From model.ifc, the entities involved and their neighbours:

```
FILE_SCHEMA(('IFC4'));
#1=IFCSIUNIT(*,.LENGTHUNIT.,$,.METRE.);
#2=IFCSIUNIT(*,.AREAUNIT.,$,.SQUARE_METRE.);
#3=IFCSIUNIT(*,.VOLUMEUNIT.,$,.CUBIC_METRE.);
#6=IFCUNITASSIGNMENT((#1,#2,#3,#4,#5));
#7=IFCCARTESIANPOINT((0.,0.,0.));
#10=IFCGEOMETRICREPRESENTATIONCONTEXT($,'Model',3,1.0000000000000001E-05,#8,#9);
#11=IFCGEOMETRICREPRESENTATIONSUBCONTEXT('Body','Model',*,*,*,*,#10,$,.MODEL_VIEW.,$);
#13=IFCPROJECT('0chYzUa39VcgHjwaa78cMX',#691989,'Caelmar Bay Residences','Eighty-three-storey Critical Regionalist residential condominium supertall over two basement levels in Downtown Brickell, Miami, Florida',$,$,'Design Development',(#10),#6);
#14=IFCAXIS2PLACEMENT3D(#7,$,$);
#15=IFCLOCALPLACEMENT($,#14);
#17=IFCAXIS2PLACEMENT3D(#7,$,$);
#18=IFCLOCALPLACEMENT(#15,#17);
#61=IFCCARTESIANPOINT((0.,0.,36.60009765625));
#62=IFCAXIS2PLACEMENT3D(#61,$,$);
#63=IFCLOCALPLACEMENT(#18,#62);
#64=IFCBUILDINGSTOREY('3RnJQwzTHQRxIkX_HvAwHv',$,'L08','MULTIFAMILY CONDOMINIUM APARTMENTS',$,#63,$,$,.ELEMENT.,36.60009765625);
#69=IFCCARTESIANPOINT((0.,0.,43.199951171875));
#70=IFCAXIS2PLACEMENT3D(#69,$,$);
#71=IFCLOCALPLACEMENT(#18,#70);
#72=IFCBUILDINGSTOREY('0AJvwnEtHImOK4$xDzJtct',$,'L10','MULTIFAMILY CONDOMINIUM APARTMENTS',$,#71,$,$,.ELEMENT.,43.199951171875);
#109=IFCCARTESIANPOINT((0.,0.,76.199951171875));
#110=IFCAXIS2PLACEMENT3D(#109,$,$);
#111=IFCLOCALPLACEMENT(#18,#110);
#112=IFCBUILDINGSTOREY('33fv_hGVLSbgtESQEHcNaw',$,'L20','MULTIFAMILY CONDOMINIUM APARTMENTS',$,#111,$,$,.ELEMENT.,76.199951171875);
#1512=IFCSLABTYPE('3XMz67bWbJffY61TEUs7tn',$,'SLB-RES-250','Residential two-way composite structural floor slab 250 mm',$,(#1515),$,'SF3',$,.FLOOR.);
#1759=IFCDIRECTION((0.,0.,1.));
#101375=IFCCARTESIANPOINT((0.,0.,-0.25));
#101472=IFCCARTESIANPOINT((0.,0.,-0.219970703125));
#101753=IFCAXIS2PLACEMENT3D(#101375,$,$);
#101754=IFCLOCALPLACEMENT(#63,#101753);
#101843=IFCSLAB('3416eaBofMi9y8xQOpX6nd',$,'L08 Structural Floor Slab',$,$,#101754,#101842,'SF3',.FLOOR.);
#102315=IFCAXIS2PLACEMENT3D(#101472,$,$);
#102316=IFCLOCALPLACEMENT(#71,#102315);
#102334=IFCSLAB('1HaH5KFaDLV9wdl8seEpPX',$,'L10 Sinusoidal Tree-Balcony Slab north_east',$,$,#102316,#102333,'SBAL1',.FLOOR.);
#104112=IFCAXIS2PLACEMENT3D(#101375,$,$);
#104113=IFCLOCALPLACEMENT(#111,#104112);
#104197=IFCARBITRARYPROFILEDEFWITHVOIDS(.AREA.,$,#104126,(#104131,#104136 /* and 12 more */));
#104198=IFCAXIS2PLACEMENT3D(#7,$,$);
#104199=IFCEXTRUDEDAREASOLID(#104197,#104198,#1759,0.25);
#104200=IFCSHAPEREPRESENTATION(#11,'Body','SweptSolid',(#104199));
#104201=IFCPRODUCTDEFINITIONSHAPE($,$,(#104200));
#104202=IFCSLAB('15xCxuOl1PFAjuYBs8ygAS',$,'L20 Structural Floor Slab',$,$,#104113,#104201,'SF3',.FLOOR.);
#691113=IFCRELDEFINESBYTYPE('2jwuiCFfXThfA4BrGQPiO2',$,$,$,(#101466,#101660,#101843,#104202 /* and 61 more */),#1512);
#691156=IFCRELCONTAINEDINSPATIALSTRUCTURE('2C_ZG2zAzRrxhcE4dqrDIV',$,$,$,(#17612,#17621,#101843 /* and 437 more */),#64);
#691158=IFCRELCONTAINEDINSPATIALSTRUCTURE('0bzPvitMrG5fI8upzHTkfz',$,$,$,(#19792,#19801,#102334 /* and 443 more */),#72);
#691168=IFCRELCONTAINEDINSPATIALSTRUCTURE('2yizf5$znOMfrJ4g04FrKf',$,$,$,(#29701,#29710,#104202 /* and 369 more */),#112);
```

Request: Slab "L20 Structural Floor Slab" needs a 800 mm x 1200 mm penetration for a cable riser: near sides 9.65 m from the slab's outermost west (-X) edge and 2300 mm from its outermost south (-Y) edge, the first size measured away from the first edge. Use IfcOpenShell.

```python
import numpy as np
import ifcopenshell
import ifcopenshell.api.feature
import ifcopenshell.api.geometry
import ifcopenshell.api.root
import ifcopenshell.geom
import ifcopenshell.util.placement
import ifcopenshell.util.representation
import ifcopenshell.util.shape
import ifcopenshell.util.unit

model = ifcopenshell.open("model.ifc")
unit_scale = ifcopenshell.util.unit.calculate_unit_scale(model)
settings = ifcopenshell.geom.settings()


def volume(element):
    """Net volume in cubic metres, openings subtracted."""
    shape = ifcopenshell.geom.create_shape(settings, element)
    return ifcopenshell.util.shape.get_volume(shape.geometry)


slab = model.by_id(104202)
before = volume(slab)

# Extent in the slab's own axes, in metres. The edges named are its -X and -Y sides.
slab_shape = ifcopenshell.geom.create_shape(settings, slab)
vertices = ifcopenshell.util.shape.get_vertices(slab_shape.geometry)
x_min, y_min, bottom = vertices.min(axis=0)
top = vertices[:, 2].max()

opening = ifcopenshell.api.root.create_entity(model, ifc_class="IfcOpeningElement", name="Cable riser opening", predefined_type="OPENING")
context = ifcopenshell.util.representation.get_context(model, "Model", "Body", "MODEL_VIEW")
width, depth = 0.8, 1.2
outline = [(0.0, 0.0), (width, 0.0), (width, depth), (0.0, depth), (0.0, 0.0)]
# Overshoot both faces by 50 mm so the cut is clean.
shape = ifcopenshell.api.geometry.add_slab_representation(
    model, context=context, depth=top - bottom + 0.1, polyline=outline
)
ifcopenshell.api.geometry.assign_representation(model, product=opening, representation=shape)

matrix = ifcopenshell.util.placement.get_local_placement(slab.ObjectPlacement)
matrix[:, 3] = matrix @ np.append(np.array([x_min + 9.65, y_min + 2.3, bottom - 0.05]) / unit_scale, 1.0)
ifcopenshell.api.geometry.edit_object_placement(model, product=opening, matrix=matrix, is_si=False)
ifcopenshell.api.feature.add_feature(model, feature=opening, element=slab)

after = volume(slab)

print(f"slab volume {before:.3f} -> {after:.3f} m3")

model.write("model_edited.ifc")
```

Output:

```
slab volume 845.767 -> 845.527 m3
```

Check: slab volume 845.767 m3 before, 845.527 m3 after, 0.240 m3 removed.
